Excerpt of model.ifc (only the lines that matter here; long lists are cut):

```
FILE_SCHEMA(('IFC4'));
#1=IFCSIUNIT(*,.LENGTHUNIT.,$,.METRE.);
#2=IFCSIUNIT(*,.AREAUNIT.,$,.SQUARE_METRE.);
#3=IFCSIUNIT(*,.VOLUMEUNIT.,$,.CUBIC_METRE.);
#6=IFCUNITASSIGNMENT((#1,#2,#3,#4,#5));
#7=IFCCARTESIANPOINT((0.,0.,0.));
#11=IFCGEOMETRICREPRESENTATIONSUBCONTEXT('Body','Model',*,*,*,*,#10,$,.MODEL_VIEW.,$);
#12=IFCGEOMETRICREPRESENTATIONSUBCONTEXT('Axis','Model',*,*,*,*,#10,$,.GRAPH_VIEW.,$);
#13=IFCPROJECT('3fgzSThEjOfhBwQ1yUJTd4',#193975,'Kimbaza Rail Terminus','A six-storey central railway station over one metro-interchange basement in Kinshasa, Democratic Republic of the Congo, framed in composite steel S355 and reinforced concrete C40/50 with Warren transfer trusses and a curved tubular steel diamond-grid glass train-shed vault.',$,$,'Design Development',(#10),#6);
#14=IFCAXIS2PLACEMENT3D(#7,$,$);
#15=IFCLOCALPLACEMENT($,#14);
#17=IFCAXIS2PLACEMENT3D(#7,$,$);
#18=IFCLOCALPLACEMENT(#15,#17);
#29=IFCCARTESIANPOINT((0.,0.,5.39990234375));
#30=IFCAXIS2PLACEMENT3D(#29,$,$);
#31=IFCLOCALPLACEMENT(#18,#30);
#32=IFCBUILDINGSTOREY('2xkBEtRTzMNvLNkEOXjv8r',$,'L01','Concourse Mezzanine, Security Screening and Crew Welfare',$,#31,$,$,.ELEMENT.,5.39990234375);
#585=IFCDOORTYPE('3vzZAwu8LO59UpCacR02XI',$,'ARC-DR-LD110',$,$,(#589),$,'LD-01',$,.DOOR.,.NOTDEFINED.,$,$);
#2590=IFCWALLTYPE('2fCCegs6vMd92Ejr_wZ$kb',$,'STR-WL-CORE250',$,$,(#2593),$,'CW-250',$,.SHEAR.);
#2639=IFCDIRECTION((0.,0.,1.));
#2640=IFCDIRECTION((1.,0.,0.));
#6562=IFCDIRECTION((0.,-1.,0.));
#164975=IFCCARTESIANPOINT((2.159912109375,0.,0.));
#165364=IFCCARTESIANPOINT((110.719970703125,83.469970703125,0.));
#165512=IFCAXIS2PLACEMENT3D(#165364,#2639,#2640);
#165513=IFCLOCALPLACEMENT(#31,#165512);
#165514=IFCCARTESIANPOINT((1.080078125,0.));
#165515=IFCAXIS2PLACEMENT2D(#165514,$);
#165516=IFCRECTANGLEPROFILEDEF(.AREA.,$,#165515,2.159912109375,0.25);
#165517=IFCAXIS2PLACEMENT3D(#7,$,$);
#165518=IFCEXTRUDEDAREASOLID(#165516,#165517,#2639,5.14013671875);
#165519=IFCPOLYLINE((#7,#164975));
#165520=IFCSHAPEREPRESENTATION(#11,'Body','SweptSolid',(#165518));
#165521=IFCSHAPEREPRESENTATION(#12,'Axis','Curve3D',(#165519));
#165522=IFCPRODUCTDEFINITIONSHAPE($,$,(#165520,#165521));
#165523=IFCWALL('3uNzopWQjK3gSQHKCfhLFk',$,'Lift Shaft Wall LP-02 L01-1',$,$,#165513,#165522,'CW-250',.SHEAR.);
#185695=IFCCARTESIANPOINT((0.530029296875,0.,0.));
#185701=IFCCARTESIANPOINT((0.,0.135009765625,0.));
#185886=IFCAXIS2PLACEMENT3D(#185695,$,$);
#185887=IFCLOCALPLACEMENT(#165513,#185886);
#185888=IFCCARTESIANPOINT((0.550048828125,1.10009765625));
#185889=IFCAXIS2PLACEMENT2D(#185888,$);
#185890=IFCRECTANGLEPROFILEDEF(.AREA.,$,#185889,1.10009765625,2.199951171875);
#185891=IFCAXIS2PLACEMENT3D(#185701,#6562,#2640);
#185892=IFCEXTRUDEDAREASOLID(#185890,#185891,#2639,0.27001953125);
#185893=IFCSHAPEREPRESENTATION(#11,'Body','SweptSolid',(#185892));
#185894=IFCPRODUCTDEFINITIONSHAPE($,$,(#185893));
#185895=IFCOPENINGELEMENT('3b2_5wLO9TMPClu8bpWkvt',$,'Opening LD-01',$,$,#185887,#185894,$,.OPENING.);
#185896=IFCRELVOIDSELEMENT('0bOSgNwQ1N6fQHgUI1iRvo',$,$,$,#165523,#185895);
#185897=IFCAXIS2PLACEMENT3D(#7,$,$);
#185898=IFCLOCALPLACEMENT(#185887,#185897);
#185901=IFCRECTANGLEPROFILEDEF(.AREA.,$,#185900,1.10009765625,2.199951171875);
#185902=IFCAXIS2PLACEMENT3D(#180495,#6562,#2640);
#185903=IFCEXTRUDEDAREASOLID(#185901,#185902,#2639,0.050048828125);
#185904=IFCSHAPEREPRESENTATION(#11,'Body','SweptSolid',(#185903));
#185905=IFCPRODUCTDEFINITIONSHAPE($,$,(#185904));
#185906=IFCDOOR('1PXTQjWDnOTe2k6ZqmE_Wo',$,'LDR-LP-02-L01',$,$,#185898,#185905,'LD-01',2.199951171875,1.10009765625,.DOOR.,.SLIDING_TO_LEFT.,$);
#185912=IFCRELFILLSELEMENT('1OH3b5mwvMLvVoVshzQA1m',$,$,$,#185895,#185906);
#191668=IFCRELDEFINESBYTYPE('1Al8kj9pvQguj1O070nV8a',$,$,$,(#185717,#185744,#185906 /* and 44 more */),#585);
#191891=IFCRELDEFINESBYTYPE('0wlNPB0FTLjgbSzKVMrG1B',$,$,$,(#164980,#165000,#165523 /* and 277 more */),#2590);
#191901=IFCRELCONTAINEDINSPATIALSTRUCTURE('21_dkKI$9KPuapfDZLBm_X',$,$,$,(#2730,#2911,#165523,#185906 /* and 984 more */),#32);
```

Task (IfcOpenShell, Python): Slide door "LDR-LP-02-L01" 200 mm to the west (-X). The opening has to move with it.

```python
import ifcopenshell
import ifcopenshell.api.geometry
import ifcopenshell.util.placement

model = ifcopenshell.open("model.ifc")

door = model.by_guid("1PXTQjWDnOTe2k6ZqmE_Wo")
opening = door.FillsVoids[0].RelatingOpeningElement
wall = opening.VoidsElements[0].RelatingBuildingElement

wall_matrix = ifcopenshell.util.placement.get_local_placement(wall.ObjectPlacement)
shift = wall_matrix[:3, 0] * -0.2
before = ifcopenshell.util.placement.get_local_placement(door.ObjectPlacement)[:3, 3].copy()

# The door is placed relative to its opening, so it follows when the opening moves.
matrix = ifcopenshell.util.placement.get_local_placement(opening.ObjectPlacement)
matrix[:3, 3] += shift
ifcopenshell.api.geometry.edit_object_placement(
    model, product=opening, matrix=matrix, is_si=False, should_transform_children=True
)

after = ifcopenshell.util.placement.get_local_placement(door.ObjectPlacement)[:3, 3]
print("door moved by", (after - before).round(3) + 0.0)

model.write("model_v2.ifc")
```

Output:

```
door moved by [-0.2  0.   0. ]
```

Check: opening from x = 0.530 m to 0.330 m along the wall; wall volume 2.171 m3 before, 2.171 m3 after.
